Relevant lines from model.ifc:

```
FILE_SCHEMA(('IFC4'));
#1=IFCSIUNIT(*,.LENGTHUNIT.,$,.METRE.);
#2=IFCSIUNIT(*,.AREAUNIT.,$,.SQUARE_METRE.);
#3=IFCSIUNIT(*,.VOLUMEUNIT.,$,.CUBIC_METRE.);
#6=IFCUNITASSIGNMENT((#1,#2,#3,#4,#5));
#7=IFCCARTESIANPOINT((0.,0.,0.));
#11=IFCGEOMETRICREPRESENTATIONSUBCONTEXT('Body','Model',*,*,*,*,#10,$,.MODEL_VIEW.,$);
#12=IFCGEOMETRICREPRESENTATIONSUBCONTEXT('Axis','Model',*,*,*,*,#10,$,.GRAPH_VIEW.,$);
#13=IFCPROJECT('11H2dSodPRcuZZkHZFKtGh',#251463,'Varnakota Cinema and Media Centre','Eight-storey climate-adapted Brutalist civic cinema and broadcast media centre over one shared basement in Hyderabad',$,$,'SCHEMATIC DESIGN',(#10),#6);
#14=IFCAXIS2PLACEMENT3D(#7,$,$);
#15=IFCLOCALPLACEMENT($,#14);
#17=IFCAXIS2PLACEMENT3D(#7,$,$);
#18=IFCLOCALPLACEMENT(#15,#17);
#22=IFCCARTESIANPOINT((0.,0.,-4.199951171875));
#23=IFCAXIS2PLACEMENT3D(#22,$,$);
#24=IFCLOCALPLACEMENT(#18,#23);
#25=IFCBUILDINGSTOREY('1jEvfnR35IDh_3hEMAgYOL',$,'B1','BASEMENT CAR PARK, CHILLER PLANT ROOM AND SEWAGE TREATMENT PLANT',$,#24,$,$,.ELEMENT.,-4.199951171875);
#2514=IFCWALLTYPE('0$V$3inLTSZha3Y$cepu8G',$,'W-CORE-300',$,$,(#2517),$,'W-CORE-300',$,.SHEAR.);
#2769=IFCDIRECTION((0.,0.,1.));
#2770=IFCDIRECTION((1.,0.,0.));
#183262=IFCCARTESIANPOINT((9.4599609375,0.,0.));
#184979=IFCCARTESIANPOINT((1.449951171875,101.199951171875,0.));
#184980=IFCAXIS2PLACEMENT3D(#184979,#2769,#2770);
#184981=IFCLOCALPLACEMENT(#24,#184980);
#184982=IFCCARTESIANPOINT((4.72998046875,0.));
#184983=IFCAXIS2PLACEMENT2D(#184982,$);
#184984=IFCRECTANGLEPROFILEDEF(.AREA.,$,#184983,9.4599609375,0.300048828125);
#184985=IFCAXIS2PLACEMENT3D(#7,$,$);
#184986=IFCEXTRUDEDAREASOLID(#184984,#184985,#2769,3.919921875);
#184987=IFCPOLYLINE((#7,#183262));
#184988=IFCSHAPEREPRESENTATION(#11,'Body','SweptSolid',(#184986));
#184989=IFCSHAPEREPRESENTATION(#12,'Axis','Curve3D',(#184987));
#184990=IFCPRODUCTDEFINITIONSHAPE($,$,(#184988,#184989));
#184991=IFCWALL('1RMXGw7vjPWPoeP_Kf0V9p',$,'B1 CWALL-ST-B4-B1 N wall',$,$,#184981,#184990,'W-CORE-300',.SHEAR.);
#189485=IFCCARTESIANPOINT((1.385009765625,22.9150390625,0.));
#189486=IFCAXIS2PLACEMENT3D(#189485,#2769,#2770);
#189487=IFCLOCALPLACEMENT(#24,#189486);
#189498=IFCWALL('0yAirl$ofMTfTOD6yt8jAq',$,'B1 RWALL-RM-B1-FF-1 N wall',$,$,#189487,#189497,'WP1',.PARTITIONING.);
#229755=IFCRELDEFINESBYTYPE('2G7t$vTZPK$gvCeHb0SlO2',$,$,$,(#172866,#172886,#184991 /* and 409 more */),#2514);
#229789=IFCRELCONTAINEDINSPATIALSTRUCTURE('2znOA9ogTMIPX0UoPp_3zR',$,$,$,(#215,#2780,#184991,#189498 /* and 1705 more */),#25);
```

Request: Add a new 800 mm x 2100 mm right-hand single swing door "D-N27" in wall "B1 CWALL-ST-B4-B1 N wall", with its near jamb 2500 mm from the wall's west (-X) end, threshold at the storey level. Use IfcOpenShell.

```python
import numpy as np
import ifcopenshell
import ifcopenshell.api.feature
import ifcopenshell.api.geometry
import ifcopenshell.api.root
import ifcopenshell.api.spatial
import ifcopenshell.geom
import ifcopenshell.util.element
import ifcopenshell.util.placement
import ifcopenshell.util.representation
import ifcopenshell.util.shape
import ifcopenshell.util.unit

model = ifcopenshell.open("model.ifc")
unit_scale = ifcopenshell.util.unit.calculate_unit_scale(model)
settings = ifcopenshell.geom.settings()


def volume(element):
    """Net volume in cubic metres, openings subtracted."""
    shape = ifcopenshell.geom.create_shape(settings, element)
    return ifcopenshell.util.shape.get_volume(shape.geometry)


wall = model.by_id(184991)
storey = ifcopenshell.util.element.get_container(wall, ifc_class="IfcBuildingStorey")
context = ifcopenshell.util.representation.get_context(model, "Model", "Body", "MODEL_VIEW")
before = volume(wall)

width, height, from_end, sill = 0.8, 2.1, 2.5, 0.0  # metres

# The wall runs along its own X axis, and the end named is its -X end.
wall_shape = ifcopenshell.geom.create_shape(settings, wall)
x, y, z = ifcopenshell.util.shape.get_vertices(wall_shape.geometry).T
start = x.min() + from_end
face, thickness = float(y.min()), float(y.max() - y.min())
wall_matrix = ifcopenshell.util.placement.get_local_placement(wall.ObjectPlacement)
level = ifcopenshell.util.placement.get_local_placement(storey.ObjectPlacement)[2, 3]


def in_wall(x, y):
    """Placement at x, y metres in the wall's axes, at sill height."""
    matrix = wall_matrix.copy()
    matrix[:, 3] = wall_matrix @ np.array([x / unit_scale, y / unit_scale, 0.0, 1.0])
    matrix[2, 3] = level + sill / unit_scale
    return matrix


# Opening: a box that overshoots both wall faces by 50 mm.
opening = ifcopenshell.api.root.create_entity(model, ifc_class="IfcOpeningElement", predefined_type="OPENING")
box = ifcopenshell.api.geometry.add_wall_representation(
    model, context=context, length=width, height=height, thickness=thickness + 0.1
)
ifcopenshell.api.geometry.assign_representation(model, product=opening, representation=box)
ifcopenshell.api.geometry.edit_object_placement(model, product=opening, matrix=in_wall(start, face - 0.05), is_si=False)
ifcopenshell.api.feature.add_feature(model, feature=opening, element=wall)

door = ifcopenshell.api.root.create_entity(model, ifc_class="IfcDoor", name="D-N27", predefined_type="DOOR")
door.OverallWidth, door.OverallHeight = width / unit_scale, height / unit_scale
door.OperationType = "SINGLE_SWING_RIGHT"
body = ifcopenshell.api.geometry.add_door_representation(
    model,
    context=context,
    overall_width=door.OverallWidth,
    overall_height=door.OverallHeight,
    operation_type="SINGLE_SWING_RIGHT",
    lining_properties={"LiningDepth": thickness / unit_scale, "ThresholdDepth": thickness / unit_scale},
)
ifcopenshell.api.geometry.assign_representation(model, product=door, representation=body)
ifcopenshell.api.spatial.assign_container(model, products=[door], relating_structure=storey)
ifcopenshell.api.feature.add_filling(model, opening=opening, element=door)

# The lining spans the wall, so the door starts at the wall face.
ifcopenshell.api.geometry.edit_object_placement(model, product=door, matrix=in_wall(start, face), is_si=False)

after = volume(wall)

print(f"wall volume {before:.3f} -> {after:.3f} m3")

model.write("model_updated.ifc")
```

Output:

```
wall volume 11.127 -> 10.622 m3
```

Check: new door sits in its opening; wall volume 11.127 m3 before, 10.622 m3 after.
